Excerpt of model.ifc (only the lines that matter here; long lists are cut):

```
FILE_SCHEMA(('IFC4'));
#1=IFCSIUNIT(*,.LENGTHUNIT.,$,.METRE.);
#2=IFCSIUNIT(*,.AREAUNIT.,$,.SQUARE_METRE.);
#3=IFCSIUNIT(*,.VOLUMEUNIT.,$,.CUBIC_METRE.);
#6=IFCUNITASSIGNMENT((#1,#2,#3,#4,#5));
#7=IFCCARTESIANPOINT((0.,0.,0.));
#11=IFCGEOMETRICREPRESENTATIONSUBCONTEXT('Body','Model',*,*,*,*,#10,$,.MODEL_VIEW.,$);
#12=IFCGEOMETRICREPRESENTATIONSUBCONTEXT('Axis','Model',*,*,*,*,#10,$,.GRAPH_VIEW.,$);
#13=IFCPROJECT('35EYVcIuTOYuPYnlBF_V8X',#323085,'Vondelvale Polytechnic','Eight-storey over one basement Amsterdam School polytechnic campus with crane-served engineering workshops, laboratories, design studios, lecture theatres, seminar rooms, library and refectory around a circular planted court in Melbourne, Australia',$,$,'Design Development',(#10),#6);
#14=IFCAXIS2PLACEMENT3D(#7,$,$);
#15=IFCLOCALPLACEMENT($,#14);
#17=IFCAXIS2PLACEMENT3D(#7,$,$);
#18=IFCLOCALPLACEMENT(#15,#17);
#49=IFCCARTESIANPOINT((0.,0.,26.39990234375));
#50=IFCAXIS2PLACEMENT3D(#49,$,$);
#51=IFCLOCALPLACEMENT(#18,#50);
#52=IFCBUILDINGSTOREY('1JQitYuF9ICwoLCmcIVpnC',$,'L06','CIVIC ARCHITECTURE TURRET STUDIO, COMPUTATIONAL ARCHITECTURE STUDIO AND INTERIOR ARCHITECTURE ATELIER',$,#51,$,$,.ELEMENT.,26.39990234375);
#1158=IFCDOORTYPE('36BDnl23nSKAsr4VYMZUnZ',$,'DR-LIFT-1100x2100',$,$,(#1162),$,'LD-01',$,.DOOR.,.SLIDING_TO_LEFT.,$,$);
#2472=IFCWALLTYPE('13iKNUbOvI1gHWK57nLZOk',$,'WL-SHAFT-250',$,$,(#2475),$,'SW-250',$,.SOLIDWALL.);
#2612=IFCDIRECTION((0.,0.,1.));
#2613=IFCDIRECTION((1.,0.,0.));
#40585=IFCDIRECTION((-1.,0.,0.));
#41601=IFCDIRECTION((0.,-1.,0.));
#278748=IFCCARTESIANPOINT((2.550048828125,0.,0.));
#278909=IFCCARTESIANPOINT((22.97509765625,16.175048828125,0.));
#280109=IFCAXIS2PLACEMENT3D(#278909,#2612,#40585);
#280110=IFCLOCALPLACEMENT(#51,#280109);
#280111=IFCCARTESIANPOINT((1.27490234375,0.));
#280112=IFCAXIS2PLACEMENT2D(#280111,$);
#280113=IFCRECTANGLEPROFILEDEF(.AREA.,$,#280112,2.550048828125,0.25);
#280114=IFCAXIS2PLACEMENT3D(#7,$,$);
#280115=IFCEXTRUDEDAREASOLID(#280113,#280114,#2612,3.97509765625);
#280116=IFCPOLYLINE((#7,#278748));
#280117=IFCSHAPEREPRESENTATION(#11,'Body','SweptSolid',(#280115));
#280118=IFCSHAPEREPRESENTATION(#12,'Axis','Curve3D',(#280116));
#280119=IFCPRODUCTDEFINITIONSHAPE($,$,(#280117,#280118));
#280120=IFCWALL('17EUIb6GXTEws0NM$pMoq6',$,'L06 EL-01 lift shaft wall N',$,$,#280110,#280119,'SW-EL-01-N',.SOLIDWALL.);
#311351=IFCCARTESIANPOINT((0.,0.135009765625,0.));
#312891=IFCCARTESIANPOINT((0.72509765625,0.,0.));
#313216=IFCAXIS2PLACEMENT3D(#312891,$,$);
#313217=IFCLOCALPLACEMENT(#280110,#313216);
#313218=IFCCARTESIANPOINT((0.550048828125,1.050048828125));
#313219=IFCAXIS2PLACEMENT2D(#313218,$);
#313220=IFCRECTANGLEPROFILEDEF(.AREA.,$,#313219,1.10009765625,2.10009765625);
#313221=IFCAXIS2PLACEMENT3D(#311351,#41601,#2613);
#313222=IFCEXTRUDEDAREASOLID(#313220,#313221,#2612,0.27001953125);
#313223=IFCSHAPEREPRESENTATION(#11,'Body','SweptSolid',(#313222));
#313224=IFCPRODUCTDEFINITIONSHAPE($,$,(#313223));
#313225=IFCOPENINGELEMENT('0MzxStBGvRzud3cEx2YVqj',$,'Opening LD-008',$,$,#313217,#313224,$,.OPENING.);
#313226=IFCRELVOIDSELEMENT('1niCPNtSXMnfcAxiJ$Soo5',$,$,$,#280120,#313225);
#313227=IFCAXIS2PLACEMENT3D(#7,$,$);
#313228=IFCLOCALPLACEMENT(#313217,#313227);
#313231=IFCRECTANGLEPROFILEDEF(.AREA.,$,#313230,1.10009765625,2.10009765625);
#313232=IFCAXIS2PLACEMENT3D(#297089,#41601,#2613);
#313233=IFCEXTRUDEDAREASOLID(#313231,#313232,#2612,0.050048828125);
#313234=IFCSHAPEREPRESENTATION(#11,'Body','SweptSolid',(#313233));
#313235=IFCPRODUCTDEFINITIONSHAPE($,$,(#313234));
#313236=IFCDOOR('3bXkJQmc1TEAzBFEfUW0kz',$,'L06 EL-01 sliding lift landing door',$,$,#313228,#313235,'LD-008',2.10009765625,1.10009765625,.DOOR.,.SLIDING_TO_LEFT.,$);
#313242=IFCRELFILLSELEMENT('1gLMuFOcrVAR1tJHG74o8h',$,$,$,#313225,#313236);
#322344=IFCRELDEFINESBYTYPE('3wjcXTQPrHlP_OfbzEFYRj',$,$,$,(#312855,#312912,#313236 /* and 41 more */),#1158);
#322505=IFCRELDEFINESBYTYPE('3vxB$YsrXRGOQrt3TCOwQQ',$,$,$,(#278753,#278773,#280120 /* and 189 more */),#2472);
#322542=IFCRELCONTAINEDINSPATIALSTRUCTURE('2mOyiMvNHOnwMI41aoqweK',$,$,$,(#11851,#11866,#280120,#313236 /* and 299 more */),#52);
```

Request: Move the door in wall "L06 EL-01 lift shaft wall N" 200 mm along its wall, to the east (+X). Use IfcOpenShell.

```python
import ifcopenshell
import ifcopenshell.api.geometry
import ifcopenshell.util.placement

model = ifcopenshell.open("model.ifc")

door = model.by_guid("3bXkJQmc1TEAzBFEfUW0kz")
opening = door.FillsVoids[0].RelatingOpeningElement
wall = opening.VoidsElements[0].RelatingBuildingElement

wall_matrix = ifcopenshell.util.placement.get_local_placement(wall.ObjectPlacement)
shift = wall_matrix[:3, 0] * -0.2
before = ifcopenshell.util.placement.get_local_placement(door.ObjectPlacement)[:3, 3].copy()

# The door is placed relative to its opening, so it follows when the opening moves.
matrix = ifcopenshell.util.placement.get_local_placement(opening.ObjectPlacement)
matrix[:3, 3] += shift
ifcopenshell.api.geometry.edit_object_placement(
    model, product=opening, matrix=matrix, is_si=False, should_transform_children=True
)

after = ifcopenshell.util.placement.get_local_placement(door.ObjectPlacement)[:3, 3]
print("door moved by", (after - before).round(3) + 0.0)

model.write("model_updated.ifc")
```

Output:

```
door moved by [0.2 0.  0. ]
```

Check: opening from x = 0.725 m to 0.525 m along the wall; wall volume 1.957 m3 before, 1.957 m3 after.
